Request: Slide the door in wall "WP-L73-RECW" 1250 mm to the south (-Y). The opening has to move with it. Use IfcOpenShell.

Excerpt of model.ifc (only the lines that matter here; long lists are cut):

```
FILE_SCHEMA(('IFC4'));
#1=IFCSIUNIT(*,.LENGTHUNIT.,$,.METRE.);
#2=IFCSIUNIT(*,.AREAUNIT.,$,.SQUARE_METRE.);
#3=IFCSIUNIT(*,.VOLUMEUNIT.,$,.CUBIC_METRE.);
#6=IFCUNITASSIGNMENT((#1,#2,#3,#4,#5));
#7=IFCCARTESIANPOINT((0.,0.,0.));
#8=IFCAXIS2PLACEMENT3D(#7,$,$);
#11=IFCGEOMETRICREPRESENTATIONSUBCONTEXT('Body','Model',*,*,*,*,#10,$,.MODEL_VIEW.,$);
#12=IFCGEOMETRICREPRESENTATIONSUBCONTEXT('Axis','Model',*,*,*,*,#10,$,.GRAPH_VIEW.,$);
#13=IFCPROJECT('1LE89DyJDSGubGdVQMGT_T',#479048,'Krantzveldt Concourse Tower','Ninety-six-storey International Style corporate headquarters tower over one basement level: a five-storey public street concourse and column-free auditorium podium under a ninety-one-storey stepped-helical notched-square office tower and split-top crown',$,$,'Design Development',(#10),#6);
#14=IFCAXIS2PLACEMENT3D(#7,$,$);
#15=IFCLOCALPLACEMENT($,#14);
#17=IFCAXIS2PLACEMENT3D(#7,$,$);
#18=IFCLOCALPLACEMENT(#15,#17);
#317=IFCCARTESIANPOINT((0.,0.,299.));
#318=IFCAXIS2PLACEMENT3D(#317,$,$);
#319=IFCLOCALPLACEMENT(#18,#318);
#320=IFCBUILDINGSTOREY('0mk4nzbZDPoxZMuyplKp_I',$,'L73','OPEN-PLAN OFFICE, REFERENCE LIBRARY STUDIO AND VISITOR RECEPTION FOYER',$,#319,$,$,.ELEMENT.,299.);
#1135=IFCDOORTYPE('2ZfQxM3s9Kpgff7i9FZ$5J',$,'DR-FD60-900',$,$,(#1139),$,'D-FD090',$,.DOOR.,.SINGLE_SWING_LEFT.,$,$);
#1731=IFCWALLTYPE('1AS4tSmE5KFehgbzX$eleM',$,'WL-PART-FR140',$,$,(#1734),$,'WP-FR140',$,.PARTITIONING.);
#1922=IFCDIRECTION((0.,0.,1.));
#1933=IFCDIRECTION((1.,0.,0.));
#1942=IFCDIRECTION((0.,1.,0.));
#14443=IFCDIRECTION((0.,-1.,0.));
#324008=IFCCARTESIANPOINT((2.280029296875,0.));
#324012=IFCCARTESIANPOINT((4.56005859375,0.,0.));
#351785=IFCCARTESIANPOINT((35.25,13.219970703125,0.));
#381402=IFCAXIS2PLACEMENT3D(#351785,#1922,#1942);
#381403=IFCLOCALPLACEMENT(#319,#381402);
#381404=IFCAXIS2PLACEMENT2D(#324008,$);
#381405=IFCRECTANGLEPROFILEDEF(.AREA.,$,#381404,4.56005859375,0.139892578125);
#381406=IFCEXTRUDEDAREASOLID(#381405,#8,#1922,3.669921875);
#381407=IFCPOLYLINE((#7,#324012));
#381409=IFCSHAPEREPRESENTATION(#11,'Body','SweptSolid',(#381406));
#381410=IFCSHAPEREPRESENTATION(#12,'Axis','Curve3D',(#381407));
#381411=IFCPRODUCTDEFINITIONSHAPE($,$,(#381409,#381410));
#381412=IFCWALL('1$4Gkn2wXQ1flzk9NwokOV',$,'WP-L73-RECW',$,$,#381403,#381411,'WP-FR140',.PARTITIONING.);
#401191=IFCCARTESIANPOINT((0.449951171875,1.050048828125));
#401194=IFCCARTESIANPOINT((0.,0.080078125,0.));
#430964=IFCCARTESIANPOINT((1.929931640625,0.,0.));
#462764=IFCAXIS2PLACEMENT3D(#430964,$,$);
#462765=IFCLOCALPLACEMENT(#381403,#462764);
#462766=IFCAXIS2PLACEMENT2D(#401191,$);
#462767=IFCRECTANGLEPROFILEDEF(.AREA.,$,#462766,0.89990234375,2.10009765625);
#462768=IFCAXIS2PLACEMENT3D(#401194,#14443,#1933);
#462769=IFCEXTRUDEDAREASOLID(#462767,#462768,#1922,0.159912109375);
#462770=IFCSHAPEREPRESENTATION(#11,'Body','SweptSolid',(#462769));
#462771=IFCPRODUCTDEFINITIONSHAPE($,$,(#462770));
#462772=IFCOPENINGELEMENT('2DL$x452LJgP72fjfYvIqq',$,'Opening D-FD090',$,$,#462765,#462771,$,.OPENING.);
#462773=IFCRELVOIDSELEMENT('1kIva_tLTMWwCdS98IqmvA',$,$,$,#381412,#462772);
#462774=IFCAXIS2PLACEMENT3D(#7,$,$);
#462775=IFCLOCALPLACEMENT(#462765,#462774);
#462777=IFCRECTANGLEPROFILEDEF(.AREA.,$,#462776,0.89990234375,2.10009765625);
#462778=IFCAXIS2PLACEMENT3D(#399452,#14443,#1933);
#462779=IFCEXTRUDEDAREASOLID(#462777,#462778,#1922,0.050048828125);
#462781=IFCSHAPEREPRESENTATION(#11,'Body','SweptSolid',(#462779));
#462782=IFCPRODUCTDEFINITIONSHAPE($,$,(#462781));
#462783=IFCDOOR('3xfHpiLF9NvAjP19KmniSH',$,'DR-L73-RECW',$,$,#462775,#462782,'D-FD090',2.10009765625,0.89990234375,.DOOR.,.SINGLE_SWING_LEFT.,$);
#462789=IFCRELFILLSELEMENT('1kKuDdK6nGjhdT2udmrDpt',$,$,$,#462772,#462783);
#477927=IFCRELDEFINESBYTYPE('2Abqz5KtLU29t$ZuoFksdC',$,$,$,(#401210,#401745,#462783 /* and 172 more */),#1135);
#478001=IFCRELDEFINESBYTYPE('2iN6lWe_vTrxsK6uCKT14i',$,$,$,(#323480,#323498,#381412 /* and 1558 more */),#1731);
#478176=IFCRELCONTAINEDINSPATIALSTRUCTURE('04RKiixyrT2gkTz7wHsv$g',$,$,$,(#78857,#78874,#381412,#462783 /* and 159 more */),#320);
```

```python
import ifcopenshell
import ifcopenshell.api.geometry
import ifcopenshell.util.placement
import ifcopenshell.util.unit

model = ifcopenshell.open("model.ifc")
unit_scale = ifcopenshell.util.unit.calculate_unit_scale(model)

door = model.by_guid("3xfHpiLF9NvAjP19KmniSH")
opening = door.FillsVoids[0].RelatingOpeningElement
wall = opening.VoidsElements[0].RelatingBuildingElement

wall_matrix = ifcopenshell.util.placement.get_local_placement(wall.ObjectPlacement)
shift = wall_matrix[:3, 0] * -1.25 / unit_scale
before = ifcopenshell.util.placement.get_local_placement(door.ObjectPlacement)[:3, 3].copy()

# The door is placed relative to its opening, so it follows when the opening moves.
matrix = ifcopenshell.util.placement.get_local_placement(opening.ObjectPlacement)
matrix[:3, 3] += shift
ifcopenshell.api.geometry.edit_object_placement(
    model, product=opening, matrix=matrix, is_si=False, should_transform_children=True
)

after = ifcopenshell.util.placement.get_local_placement(door.ObjectPlacement)[:3, 3]
print("door moved by", (after - before).round(3) + 0.0)

model.write("model_edited.ifc")
```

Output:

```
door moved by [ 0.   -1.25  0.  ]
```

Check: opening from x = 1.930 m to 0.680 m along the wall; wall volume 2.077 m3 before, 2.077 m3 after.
